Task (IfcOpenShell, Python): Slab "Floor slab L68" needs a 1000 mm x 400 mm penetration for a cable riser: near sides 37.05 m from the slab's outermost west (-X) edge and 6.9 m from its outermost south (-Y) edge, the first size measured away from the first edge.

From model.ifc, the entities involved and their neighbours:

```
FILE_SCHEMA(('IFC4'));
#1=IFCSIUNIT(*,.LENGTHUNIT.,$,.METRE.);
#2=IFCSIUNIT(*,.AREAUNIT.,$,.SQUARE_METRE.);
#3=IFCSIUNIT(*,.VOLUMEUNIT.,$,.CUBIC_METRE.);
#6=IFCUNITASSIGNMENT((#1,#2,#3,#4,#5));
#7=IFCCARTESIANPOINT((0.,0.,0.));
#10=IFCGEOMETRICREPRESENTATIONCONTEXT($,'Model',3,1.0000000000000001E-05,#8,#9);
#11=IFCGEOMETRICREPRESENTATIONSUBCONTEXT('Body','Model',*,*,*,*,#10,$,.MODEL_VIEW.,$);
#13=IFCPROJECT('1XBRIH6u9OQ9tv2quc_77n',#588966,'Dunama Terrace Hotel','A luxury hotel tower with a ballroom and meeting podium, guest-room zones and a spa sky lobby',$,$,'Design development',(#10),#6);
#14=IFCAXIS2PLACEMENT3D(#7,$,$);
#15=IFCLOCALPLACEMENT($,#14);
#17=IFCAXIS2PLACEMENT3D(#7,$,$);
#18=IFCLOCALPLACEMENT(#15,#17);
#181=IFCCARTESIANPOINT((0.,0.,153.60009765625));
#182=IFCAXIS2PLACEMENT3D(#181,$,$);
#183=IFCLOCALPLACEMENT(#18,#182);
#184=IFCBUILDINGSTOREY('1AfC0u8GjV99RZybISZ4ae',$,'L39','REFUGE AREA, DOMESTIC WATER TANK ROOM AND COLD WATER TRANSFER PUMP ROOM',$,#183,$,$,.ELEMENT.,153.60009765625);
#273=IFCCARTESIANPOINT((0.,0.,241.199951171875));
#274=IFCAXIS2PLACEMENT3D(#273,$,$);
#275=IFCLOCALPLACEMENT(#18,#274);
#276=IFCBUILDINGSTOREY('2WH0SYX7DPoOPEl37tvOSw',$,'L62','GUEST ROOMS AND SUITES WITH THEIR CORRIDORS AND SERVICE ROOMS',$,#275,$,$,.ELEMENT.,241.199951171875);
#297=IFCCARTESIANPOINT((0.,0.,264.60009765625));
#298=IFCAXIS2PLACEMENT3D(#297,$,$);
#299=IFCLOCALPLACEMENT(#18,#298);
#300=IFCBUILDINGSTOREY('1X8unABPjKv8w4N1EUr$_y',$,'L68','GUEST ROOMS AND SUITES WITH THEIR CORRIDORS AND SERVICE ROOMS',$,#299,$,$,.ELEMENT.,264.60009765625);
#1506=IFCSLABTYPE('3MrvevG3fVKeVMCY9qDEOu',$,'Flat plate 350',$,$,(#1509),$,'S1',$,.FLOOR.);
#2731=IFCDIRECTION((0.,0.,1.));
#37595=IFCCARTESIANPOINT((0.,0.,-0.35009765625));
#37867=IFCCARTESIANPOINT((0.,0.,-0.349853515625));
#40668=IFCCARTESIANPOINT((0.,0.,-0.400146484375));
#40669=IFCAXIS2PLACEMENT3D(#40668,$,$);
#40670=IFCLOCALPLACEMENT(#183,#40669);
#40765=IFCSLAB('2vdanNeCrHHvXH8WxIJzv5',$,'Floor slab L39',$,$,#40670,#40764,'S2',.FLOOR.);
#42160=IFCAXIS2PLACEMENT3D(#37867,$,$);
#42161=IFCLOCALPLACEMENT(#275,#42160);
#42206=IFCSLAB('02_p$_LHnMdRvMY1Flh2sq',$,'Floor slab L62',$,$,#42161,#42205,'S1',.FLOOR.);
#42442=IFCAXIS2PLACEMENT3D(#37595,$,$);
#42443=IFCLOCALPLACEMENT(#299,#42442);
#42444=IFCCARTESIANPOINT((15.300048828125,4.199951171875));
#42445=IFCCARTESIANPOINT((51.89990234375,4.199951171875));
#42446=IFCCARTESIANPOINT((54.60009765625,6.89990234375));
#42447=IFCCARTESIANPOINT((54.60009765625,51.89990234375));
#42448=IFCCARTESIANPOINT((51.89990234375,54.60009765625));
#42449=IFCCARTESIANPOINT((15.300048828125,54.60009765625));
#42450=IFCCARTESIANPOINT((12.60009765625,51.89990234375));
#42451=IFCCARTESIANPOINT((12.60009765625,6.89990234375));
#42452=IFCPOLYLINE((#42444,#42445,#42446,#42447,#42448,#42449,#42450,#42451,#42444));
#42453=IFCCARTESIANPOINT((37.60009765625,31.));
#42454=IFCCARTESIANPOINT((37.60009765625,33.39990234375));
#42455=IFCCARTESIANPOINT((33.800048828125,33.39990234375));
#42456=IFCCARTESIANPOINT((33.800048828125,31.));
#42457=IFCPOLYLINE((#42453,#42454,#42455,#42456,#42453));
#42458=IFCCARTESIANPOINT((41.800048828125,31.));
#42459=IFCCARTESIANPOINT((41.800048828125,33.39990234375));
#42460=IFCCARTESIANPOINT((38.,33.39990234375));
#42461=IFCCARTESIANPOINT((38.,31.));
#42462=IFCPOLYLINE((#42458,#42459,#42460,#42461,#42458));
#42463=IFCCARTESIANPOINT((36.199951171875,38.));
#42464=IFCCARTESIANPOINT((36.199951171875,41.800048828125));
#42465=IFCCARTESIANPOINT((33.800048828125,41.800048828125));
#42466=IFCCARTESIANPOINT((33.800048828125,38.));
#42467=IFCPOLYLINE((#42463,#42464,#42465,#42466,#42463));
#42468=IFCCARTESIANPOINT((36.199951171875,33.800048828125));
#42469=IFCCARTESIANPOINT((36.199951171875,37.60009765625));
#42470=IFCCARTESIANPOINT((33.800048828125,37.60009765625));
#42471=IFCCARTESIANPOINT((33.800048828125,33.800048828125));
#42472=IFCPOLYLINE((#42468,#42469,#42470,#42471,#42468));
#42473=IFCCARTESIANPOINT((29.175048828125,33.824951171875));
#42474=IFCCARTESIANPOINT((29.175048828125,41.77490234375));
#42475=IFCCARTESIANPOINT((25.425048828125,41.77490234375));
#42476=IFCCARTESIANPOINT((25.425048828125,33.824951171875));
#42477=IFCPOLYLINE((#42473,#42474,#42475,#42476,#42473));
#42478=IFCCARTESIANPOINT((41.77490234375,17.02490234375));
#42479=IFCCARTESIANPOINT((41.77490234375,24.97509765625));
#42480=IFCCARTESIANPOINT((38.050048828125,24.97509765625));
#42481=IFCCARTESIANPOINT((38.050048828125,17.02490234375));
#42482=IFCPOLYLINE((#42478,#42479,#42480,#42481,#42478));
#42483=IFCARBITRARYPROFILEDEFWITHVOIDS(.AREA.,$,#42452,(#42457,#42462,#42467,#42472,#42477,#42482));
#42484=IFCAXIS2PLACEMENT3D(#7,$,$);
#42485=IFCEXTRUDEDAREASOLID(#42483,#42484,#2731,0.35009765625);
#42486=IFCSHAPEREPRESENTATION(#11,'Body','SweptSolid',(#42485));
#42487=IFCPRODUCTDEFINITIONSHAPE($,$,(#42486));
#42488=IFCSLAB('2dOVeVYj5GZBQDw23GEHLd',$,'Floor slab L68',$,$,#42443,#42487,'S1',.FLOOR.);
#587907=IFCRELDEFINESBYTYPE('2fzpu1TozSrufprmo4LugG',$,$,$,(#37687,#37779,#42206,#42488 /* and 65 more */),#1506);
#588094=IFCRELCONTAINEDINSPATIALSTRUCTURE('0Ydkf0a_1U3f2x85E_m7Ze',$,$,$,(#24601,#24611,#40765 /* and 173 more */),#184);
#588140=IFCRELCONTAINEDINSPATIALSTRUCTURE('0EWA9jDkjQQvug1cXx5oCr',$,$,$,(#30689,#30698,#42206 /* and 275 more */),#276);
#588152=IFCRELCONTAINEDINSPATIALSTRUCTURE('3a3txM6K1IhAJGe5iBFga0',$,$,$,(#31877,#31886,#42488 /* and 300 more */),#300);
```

```python
import numpy as np
import ifcopenshell
import ifcopenshell.api.feature
import ifcopenshell.api.geometry
import ifcopenshell.api.root
import ifcopenshell.geom
import ifcopenshell.util.placement
import ifcopenshell.util.representation
import ifcopenshell.util.shape
import ifcopenshell.util.unit

model = ifcopenshell.open("model.ifc")
unit_scale = ifcopenshell.util.unit.calculate_unit_scale(model)
settings = ifcopenshell.geom.settings()


def volume(element):
    """Net volume in cubic metres, openings subtracted."""
    shape = ifcopenshell.geom.create_shape(settings, element)
    return ifcopenshell.util.shape.get_volume(shape.geometry)


slab = model.by_id(42488)
before = volume(slab)

# Extent in the slab's own axes, in metres. The edges named are its -X and -Y sides.
slab_shape = ifcopenshell.geom.create_shape(settings, slab)
vertices = ifcopenshell.util.shape.get_vertices(slab_shape.geometry)
x_min, y_min, bottom = vertices.min(axis=0)
top = vertices[:, 2].max()

opening = ifcopenshell.api.root.create_entity(model, ifc_class="IfcOpeningElement", name="Cable riser opening", predefined_type="OPENING")
context = ifcopenshell.util.representation.get_context(model, "Model", "Body", "MODEL_VIEW")
width, depth = 1, 0.4
outline = [(0.0, 0.0), (width, 0.0), (width, depth), (0.0, depth), (0.0, 0.0)]
# Overshoot both faces by 50 mm so the cut is clean.
shape = ifcopenshell.api.geometry.add_slab_representation(
    model, context=context, depth=top - bottom + 0.1, polyline=outline
)
ifcopenshell.api.geometry.assign_representation(model, product=opening, representation=shape)

matrix = ifcopenshell.util.placement.get_local_placement(slab.ObjectPlacement)
matrix[:, 3] = matrix @ np.append(np.array([x_min + 37.05, y_min + 6.9, bottom - 0.05]) / unit_scale, 1.0)
ifcopenshell.api.geometry.edit_object_placement(model, product=opening, matrix=matrix, is_si=False)
ifcopenshell.api.feature.add_feature(model, feature=opening, element=slab)

after = volume(slab)

print(f"slab volume {before:.3f} -> {after:.3f} m3")

model.write("model_v2.ifc")
```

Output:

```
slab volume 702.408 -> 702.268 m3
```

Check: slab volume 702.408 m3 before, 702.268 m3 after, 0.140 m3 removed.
